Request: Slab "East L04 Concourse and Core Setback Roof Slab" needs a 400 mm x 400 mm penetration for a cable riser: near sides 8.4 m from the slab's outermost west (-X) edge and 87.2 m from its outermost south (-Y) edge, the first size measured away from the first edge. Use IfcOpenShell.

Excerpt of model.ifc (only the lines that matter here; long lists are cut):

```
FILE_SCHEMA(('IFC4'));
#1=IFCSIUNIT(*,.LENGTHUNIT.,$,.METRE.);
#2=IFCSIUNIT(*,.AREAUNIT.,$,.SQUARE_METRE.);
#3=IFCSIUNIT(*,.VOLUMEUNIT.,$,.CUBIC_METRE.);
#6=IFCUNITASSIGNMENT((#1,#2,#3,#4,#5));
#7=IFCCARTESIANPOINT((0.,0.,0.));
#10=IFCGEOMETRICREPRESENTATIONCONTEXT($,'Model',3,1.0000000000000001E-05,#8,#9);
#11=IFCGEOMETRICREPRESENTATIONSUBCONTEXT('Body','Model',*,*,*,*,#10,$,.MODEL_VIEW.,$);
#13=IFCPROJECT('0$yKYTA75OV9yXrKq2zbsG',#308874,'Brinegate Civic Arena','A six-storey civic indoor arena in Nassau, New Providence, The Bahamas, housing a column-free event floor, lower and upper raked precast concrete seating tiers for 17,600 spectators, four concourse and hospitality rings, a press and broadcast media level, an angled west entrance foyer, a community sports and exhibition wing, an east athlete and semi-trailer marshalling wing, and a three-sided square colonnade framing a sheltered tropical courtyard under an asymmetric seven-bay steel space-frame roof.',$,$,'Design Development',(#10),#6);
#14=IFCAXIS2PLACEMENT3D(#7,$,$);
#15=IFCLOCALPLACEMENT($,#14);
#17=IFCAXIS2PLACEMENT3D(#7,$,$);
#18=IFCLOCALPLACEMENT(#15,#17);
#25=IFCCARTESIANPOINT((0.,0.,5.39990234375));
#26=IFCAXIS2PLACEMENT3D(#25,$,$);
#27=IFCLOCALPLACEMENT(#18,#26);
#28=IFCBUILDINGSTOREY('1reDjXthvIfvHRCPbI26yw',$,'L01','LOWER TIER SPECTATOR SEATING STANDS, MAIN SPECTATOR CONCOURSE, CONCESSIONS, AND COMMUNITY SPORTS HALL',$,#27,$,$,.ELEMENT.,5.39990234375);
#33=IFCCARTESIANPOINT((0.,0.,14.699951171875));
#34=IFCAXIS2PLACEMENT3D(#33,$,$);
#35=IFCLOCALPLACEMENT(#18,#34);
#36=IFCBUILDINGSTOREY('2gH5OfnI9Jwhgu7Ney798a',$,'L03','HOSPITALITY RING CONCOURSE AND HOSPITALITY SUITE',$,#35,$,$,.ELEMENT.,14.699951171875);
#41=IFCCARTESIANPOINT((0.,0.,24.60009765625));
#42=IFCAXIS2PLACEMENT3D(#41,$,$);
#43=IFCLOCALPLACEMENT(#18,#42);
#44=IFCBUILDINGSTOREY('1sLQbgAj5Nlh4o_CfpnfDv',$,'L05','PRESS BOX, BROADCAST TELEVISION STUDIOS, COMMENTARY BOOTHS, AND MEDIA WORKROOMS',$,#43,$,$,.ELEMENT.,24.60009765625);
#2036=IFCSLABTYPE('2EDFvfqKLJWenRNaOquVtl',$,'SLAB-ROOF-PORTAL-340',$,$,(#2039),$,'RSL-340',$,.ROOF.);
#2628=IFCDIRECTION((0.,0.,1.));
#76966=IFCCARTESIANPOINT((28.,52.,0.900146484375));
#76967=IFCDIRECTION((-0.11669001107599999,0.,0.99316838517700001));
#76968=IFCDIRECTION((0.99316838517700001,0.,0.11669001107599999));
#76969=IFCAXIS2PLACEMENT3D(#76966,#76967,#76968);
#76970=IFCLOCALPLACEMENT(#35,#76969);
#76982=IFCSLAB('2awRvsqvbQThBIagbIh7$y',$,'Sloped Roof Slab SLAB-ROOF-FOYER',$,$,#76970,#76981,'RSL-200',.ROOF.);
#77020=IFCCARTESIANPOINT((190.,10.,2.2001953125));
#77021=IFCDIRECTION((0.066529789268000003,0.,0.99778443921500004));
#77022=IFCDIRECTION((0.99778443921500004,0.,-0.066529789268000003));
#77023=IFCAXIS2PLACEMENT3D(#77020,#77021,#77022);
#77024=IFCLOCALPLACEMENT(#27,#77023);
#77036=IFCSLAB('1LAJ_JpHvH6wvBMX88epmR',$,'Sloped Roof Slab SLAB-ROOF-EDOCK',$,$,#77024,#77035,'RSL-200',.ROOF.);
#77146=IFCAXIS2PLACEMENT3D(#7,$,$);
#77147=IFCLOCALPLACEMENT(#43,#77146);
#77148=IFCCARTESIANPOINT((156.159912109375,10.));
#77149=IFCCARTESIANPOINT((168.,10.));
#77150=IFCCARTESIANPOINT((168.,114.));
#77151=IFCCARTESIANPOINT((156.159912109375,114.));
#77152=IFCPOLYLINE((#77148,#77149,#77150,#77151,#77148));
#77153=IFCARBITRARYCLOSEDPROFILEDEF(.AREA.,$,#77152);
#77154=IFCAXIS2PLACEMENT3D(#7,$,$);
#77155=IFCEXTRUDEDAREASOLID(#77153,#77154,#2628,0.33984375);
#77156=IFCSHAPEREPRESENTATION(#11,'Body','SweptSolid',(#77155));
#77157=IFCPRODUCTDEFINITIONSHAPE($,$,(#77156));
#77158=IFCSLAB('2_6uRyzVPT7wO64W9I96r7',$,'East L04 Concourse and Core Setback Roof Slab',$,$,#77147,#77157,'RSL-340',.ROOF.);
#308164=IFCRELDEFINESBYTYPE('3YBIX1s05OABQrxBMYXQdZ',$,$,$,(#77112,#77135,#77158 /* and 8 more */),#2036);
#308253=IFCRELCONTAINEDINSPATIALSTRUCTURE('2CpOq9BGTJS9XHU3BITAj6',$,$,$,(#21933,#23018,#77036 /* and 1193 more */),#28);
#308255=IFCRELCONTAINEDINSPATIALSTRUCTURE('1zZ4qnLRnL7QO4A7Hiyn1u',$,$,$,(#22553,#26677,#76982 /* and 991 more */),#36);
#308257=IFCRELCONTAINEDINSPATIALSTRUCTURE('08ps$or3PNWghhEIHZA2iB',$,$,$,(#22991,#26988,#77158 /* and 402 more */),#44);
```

```python
import numpy as np
import ifcopenshell
import ifcopenshell.api.feature
import ifcopenshell.api.geometry
import ifcopenshell.api.root
import ifcopenshell.geom
import ifcopenshell.util.placement
import ifcopenshell.util.representation
import ifcopenshell.util.shape
import ifcopenshell.util.unit

model = ifcopenshell.open("model.ifc")
unit_scale = ifcopenshell.util.unit.calculate_unit_scale(model)
settings = ifcopenshell.geom.settings()


def volume(element):
    """Net volume in cubic metres, openings subtracted."""
    shape = ifcopenshell.geom.create_shape(settings, element)
    return ifcopenshell.util.shape.get_volume(shape.geometry)


slab = model.by_guid("2_6uRyzVPT7wO64W9I96r7")
before = volume(slab)

# Extent in the slab's own axes, in metres. The edges named are its -X and -Y sides.
slab_shape = ifcopenshell.geom.create_shape(settings, slab)
vertices = ifcopenshell.util.shape.get_vertices(slab_shape.geometry)
x_min, y_min, bottom = vertices.min(axis=0)
top = vertices[:, 2].max()

opening = ifcopenshell.api.root.create_entity(model, ifc_class="IfcOpeningElement", name="Cable riser opening", predefined_type="OPENING")
context = ifcopenshell.util.representation.get_context(model, "Model", "Body", "MODEL_VIEW")
width, depth = 0.4, 0.4
outline = [(0.0, 0.0), (width, 0.0), (width, depth), (0.0, depth), (0.0, 0.0)]
# Overshoot both faces by 50 mm so the cut is clean.
shape = ifcopenshell.api.geometry.add_slab_representation(
    model, context=context, depth=top - bottom + 0.1, polyline=outline
)
ifcopenshell.api.geometry.assign_representation(model, product=opening, representation=shape)

matrix = ifcopenshell.util.placement.get_local_placement(slab.ObjectPlacement)
matrix[:, 3] = matrix @ np.append(np.array([x_min + 8.4, y_min + 87.2, bottom - 0.05]) / unit_scale, 1.0)
ifcopenshell.api.geometry.edit_object_placement(model, product=opening, matrix=matrix, is_si=False)
ifcopenshell.api.feature.add_feature(model, feature=opening, element=slab)

after = volume(slab)

print(f"slab volume {before:.3f} -> {after:.3f} m3")

model.write("model-out.ifc")
```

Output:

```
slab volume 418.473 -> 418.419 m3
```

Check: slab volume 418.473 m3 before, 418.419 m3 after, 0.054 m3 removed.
